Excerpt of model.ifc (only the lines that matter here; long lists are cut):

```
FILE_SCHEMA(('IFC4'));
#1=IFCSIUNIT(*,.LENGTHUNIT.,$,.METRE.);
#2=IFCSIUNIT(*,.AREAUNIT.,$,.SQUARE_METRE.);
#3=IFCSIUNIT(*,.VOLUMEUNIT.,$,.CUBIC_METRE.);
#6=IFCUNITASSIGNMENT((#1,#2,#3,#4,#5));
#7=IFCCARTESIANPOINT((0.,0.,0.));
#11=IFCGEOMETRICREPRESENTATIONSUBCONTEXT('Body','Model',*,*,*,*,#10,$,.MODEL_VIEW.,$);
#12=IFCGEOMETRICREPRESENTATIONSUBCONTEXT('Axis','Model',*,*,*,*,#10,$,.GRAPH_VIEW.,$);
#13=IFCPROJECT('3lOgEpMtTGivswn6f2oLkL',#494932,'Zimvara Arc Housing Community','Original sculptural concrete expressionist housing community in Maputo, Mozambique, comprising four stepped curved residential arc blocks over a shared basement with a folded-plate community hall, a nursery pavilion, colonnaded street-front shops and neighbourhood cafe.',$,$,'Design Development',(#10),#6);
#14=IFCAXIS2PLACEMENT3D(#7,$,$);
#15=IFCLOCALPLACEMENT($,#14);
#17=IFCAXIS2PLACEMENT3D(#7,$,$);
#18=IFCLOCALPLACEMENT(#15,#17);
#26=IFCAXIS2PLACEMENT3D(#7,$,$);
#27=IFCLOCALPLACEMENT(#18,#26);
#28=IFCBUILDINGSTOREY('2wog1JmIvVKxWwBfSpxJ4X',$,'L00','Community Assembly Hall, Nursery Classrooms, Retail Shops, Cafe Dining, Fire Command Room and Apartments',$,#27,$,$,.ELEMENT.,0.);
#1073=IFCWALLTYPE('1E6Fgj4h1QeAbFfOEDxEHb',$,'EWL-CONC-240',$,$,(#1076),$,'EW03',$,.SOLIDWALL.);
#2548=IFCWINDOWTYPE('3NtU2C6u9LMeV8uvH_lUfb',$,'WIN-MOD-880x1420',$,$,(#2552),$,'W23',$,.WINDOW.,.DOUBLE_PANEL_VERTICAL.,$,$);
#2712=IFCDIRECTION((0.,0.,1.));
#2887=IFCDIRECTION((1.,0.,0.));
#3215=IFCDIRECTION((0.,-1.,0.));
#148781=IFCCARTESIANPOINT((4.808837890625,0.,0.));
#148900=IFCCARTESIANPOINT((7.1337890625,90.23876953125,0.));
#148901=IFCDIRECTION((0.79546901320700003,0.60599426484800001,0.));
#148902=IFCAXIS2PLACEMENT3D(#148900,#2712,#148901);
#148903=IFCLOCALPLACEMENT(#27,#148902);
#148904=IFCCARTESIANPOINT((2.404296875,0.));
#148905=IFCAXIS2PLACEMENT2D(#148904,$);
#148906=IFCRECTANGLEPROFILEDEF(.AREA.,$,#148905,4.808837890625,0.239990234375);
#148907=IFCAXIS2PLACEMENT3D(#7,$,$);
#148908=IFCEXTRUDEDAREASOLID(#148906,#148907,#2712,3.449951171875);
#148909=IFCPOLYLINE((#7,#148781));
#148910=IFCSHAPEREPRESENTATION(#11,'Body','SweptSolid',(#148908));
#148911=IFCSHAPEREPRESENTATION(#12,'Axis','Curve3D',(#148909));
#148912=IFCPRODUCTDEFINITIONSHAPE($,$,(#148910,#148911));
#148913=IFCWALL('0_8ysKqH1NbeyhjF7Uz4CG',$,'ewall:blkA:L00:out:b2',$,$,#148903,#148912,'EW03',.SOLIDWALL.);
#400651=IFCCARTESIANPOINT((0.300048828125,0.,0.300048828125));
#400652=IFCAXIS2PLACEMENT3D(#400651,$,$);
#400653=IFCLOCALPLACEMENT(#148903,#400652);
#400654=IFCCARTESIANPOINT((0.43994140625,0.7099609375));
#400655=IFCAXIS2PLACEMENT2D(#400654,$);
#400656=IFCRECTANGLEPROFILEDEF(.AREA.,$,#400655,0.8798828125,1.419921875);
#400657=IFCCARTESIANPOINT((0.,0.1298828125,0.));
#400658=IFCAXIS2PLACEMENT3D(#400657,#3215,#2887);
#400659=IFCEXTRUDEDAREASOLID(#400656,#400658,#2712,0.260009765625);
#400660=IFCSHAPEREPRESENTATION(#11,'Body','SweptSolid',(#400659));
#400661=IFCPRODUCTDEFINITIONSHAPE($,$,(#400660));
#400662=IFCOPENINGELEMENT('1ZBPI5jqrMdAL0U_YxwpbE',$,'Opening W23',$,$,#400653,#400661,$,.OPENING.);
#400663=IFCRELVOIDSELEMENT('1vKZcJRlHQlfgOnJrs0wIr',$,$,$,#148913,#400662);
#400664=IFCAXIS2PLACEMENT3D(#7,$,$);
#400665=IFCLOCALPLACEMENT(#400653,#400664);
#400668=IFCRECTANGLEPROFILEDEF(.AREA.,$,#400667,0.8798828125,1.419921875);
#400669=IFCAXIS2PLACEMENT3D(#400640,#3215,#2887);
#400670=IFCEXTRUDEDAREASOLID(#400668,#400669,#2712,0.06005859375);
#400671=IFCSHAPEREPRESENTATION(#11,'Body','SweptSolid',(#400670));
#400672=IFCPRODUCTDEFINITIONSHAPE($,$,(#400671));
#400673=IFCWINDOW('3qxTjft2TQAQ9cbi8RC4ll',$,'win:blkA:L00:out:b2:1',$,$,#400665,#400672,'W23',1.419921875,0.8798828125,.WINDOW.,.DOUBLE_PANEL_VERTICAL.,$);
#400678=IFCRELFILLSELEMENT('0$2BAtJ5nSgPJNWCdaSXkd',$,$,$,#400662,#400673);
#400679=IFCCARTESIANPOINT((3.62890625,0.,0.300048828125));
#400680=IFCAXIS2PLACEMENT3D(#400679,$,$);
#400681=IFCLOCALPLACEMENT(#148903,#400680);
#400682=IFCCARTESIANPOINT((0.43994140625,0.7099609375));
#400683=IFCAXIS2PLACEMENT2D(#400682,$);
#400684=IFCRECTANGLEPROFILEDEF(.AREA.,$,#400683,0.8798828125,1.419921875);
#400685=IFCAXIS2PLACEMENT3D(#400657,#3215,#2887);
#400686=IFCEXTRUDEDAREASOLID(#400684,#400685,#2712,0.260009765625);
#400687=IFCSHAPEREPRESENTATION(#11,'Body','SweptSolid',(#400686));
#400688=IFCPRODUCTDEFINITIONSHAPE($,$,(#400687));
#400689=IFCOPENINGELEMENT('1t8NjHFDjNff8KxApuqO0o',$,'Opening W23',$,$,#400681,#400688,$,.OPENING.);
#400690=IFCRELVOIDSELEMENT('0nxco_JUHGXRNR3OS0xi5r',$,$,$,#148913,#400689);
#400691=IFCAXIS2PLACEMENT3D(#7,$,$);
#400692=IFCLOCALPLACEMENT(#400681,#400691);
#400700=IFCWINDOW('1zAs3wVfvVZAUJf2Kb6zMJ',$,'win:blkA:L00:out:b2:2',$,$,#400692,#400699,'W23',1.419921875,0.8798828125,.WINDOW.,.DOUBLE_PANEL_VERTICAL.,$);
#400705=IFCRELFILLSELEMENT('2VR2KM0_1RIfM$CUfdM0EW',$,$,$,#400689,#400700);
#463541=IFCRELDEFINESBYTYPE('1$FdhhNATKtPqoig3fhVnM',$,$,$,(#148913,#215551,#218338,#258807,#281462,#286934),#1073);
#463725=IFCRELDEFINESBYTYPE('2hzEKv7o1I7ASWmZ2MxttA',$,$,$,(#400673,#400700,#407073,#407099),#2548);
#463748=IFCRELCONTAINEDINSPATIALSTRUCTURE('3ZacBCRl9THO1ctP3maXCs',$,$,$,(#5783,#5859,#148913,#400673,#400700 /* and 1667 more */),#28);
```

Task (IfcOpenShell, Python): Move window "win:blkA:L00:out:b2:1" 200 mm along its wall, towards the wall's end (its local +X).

```python
import ifcopenshell
import ifcopenshell.api.geometry
import ifcopenshell.util.placement

model = ifcopenshell.open("model.ifc")

window = model.by_id(400673)
opening = window.FillsVoids[0].RelatingOpeningElement
wall = opening.VoidsElements[0].RelatingBuildingElement

wall_matrix = ifcopenshell.util.placement.get_local_placement(wall.ObjectPlacement)
shift = wall_matrix[:3, 0] * 0.2
before = ifcopenshell.util.placement.get_local_placement(window.ObjectPlacement)[:3, 3].copy()

# The window is placed relative to its opening, so it follows when the opening moves.
matrix = ifcopenshell.util.placement.get_local_placement(opening.ObjectPlacement)
matrix[:3, 3] += shift
ifcopenshell.api.geometry.edit_object_placement(
    model, product=opening, matrix=matrix, is_si=False, should_transform_children=True
)

after = ifcopenshell.util.placement.get_local_placement(window.ObjectPlacement)[:3, 3]
print("window moved by", (after - before).round(3) + 0.0)

model.write("model_edited.ifc")
```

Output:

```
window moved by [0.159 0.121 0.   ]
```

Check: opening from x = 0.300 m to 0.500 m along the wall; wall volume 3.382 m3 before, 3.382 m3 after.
